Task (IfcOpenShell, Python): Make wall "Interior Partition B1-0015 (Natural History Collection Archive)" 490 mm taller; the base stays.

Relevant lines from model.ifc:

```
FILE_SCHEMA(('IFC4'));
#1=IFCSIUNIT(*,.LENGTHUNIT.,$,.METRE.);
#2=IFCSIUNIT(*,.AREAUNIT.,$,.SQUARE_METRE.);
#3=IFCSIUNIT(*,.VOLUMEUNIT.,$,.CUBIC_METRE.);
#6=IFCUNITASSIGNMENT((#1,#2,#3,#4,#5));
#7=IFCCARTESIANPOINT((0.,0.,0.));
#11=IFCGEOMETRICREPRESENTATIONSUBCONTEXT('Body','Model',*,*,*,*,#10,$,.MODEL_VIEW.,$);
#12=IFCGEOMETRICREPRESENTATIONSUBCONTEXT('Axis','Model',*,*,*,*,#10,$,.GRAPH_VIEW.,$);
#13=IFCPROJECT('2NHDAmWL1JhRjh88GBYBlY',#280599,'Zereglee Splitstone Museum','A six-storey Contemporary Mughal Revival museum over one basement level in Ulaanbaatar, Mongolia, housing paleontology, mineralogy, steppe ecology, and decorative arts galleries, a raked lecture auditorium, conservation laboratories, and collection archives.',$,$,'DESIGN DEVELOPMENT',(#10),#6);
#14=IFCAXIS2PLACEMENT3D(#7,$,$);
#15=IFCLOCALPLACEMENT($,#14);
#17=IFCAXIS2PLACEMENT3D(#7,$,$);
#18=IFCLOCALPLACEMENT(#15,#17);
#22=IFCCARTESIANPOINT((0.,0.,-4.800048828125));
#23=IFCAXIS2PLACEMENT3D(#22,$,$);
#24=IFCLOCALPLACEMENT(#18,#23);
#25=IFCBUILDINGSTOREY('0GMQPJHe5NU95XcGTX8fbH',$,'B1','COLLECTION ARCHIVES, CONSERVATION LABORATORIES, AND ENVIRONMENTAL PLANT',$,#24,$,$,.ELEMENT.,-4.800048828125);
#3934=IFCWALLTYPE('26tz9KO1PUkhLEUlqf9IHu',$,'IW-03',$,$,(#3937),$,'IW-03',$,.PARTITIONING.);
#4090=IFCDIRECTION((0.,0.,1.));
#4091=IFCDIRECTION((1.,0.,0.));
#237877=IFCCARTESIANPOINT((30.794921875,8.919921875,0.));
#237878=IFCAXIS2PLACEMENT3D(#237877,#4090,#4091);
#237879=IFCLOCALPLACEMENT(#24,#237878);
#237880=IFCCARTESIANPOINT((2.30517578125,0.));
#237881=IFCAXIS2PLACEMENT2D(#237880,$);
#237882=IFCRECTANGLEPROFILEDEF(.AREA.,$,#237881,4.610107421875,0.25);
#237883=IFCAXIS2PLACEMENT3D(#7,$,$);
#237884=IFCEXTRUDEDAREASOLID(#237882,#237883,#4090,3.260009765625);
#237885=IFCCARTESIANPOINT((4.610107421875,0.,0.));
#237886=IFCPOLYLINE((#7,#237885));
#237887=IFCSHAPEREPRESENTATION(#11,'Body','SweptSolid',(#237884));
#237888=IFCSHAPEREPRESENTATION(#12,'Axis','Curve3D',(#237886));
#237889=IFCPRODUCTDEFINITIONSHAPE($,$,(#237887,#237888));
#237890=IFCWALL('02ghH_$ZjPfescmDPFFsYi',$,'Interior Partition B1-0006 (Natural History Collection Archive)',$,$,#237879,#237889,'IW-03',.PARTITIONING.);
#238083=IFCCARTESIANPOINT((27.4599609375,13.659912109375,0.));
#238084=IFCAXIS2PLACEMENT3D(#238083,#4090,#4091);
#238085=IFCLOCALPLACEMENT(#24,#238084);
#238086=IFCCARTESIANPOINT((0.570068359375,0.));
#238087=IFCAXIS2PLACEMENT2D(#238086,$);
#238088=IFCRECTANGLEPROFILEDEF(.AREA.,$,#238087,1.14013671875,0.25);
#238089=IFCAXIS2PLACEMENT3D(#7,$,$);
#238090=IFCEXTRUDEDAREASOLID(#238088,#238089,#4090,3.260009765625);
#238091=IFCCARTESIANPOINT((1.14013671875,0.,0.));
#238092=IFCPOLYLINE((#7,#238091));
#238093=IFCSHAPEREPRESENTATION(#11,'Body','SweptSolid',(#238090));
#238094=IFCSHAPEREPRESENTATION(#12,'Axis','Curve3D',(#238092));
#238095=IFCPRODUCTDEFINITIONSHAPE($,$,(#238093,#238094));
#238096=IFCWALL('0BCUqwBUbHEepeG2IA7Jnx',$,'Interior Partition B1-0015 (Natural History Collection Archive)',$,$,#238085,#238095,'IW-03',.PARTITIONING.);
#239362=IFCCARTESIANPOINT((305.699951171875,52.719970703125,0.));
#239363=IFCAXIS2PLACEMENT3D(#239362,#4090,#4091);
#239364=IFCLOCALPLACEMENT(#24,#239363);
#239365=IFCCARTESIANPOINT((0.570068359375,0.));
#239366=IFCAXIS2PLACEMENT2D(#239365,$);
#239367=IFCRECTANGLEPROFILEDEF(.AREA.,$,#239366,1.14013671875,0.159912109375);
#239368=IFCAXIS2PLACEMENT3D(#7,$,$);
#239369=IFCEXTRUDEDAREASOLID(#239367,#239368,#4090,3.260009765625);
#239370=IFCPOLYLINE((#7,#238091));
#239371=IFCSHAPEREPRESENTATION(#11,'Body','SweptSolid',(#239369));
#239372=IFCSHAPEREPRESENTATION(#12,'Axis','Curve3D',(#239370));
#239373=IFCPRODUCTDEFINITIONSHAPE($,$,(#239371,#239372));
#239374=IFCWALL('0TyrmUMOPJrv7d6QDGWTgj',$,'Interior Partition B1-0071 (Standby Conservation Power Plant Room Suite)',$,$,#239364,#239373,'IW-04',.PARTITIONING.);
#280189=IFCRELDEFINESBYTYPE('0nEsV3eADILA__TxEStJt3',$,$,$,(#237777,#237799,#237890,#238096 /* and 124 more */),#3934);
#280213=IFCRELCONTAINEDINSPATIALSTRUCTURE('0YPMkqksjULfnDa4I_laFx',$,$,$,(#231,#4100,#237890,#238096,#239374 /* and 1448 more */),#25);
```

```python
import ifcopenshell
import ifcopenshell.geom
import ifcopenshell.util.representation
import ifcopenshell.util.shape

model = ifcopenshell.open("model.ifc")
settings = ifcopenshell.geom.settings()


def volume(element):
    """Net volume in cubic metres, openings subtracted."""
    shape = ifcopenshell.geom.create_shape(settings, element)
    return ifcopenshell.util.shape.get_volume(shape.geometry)


wall = model.by_id(238096)
before = volume(wall)

body = ifcopenshell.util.representation.get_representation(wall, "Model", "Body")
solid = body.Items[0]
old_height = solid.Depth
solid.Depth += 0.49
after = volume(wall)

print(f"height {old_height:g} -> {solid.Depth:g}, volume {before:.3f} -> {after:.3f} m3")

model.write("model_v2.ifc")
```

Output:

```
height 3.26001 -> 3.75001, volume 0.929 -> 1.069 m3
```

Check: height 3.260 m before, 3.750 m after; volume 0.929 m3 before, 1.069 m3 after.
